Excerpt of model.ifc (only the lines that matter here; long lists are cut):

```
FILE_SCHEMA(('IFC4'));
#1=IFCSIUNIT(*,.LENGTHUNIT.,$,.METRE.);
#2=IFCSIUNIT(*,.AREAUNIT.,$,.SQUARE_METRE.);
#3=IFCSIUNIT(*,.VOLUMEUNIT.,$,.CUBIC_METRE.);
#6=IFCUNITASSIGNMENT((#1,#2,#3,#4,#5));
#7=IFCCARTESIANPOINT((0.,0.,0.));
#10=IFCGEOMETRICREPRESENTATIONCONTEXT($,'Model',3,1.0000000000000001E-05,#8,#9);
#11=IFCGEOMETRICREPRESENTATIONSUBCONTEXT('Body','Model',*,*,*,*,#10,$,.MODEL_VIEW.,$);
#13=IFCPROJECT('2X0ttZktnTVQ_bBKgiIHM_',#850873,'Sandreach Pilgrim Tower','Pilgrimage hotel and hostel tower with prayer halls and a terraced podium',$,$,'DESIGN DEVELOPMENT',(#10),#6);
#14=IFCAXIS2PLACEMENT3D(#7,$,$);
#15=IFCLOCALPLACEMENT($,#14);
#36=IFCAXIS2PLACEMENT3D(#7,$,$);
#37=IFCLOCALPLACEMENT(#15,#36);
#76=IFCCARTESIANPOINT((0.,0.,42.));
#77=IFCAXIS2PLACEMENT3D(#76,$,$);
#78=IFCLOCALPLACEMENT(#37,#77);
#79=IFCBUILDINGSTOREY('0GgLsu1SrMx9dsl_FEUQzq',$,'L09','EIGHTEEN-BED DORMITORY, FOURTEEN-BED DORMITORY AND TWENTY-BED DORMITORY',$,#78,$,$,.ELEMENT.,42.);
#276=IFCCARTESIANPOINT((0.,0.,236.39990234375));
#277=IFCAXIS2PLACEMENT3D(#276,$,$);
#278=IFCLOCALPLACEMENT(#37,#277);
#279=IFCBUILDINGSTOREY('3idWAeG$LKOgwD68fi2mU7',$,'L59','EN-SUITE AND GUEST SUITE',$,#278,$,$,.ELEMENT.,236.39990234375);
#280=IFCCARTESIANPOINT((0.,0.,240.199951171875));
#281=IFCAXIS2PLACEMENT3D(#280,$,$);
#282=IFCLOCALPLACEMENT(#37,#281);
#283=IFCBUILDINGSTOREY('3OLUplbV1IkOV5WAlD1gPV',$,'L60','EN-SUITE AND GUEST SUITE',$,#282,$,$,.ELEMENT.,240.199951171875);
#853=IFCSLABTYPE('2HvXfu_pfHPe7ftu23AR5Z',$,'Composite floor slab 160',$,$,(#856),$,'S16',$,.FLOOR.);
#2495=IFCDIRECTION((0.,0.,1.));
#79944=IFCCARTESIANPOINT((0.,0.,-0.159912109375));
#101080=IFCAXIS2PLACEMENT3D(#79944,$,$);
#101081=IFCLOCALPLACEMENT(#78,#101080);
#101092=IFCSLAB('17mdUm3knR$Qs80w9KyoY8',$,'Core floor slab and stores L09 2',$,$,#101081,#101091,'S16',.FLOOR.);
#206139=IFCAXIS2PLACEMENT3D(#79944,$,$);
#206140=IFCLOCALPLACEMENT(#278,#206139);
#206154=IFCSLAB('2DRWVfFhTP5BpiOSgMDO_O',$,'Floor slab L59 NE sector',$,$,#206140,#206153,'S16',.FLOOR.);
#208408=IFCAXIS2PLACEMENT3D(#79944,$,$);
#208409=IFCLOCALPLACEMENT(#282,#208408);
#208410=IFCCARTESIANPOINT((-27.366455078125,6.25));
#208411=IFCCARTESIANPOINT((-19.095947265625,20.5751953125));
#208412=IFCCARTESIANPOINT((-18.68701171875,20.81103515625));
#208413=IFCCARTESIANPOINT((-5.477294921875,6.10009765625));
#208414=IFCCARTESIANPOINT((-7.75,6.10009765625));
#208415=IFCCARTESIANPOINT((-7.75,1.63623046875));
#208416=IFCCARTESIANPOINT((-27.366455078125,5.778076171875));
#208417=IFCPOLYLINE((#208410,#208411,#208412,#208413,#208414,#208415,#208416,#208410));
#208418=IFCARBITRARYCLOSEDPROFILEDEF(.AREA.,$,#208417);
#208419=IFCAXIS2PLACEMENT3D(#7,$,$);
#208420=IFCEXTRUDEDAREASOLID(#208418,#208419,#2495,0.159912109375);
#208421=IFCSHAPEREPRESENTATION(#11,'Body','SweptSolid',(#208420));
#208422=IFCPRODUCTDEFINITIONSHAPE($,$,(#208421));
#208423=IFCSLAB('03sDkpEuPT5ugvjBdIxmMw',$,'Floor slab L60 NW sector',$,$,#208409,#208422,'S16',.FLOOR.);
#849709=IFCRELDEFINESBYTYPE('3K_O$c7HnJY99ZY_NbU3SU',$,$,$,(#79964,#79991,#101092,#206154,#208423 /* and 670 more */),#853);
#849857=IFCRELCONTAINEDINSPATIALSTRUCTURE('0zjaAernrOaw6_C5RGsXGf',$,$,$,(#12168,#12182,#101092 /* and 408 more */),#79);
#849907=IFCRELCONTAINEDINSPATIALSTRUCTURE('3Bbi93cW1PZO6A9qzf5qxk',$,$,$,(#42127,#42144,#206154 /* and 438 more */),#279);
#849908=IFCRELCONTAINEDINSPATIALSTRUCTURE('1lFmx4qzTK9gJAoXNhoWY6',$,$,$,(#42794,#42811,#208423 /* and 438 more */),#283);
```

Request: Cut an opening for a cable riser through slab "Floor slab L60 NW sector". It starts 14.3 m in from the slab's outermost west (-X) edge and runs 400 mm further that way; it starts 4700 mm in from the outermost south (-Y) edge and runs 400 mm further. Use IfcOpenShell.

```python
import numpy as np
import ifcopenshell
import ifcopenshell.api.feature
import ifcopenshell.api.geometry
import ifcopenshell.api.root
import ifcopenshell.geom
import ifcopenshell.util.placement
import ifcopenshell.util.representation
import ifcopenshell.util.shape
import ifcopenshell.util.unit

model = ifcopenshell.open("model.ifc")
unit_scale = ifcopenshell.util.unit.calculate_unit_scale(model)
settings = ifcopenshell.geom.settings()


def volume(element):
    """Net volume in cubic metres, openings subtracted."""
    shape = ifcopenshell.geom.create_shape(settings, element)
    return ifcopenshell.util.shape.get_volume(shape.geometry)


slab = model.by_id(208423)
before = volume(slab)

# Extent in the slab's own axes, in metres. The edges named are its -X and -Y sides.
slab_shape = ifcopenshell.geom.create_shape(settings, slab)
vertices = ifcopenshell.util.shape.get_vertices(slab_shape.geometry)
x_min, y_min, bottom = vertices.min(axis=0)
top = vertices[:, 2].max()

opening = ifcopenshell.api.root.create_entity(model, ifc_class="IfcOpeningElement", name="Cable riser opening", predefined_type="OPENING")
context = ifcopenshell.util.representation.get_context(model, "Model", "Body", "MODEL_VIEW")
width, depth = 0.4, 0.4
outline = [(0.0, 0.0), (width, 0.0), (width, depth), (0.0, depth), (0.0, 0.0)]
# Overshoot both faces by 50 mm so the cut is clean.
shape = ifcopenshell.api.geometry.add_slab_representation(
    model, context=context, depth=top - bottom + 0.1, polyline=outline
)
ifcopenshell.api.geometry.assign_representation(model, product=opening, representation=shape)

matrix = ifcopenshell.util.placement.get_local_placement(slab.ObjectPlacement)
matrix[:, 3] = matrix @ np.append(np.array([x_min + 14.3, y_min + 4.7, bottom - 0.05]) / unit_scale, 1.0)
ifcopenshell.api.geometry.edit_object_placement(model, product=opening, matrix=matrix, is_si=False)
ifcopenshell.api.feature.add_feature(model, feature=opening, element=slab)

after = volume(slab)

print(f"slab volume {before:.3f} -> {after:.3f} m3")

model.write("model_v2.ifc")
```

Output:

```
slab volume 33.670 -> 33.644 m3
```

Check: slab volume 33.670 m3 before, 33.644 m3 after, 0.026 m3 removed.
